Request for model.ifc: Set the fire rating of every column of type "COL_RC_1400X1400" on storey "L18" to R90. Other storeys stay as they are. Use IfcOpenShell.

First a look at what the model holds.

```python
import ifcopenshell
import ifcopenshell.util.element

model = ifcopenshell.open("model.ifc")
print(model.schema)
storey = next(s for s in model.by_type("IfcBuildingStorey") if s.Name == "L18")
columns = [e for e in ifcopenshell.util.element.get_decomposition(storey) if e.is_a("IfcColumn")]
seen = {}
for e in columns:
    element_type = ifcopenshell.util.element.get_type(e)
    key = (element_type.Name if element_type != e and element_type else None, ifcopenshell.util.element.get_pset(e, "Pset_ColumnCommon", "FireRating"))
    seen[key] = seen.get(key, 0) + 1
for (name, value), count in sorted(seen.items(), key=str):
    print(count, "x", name, "|", value)
```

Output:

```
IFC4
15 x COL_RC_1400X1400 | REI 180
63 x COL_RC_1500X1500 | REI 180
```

```python
import ifcopenshell
import ifcopenshell.api.pset
import ifcopenshell.util.element

model = ifcopenshell.open("model.ifc")

storey = next(s for s in model.by_type("IfcBuildingStorey") if s.Name == "L18")
columns = [e for e in ifcopenshell.util.element.get_decomposition(storey) if e.is_a("IfcColumn")]

count = 0
for e in columns:
    element_type = ifcopenshell.util.element.get_type(e)
    if element_type in (None, e) or element_type.Name != "COL_RC_1400X1400":
        continue
    found = ifcopenshell.util.element.get_pset(e, "Pset_ColumnCommon", should_inherit=False)
    if found:
        pset = model.by_id(found["id"])
        if len(ifcopenshell.util.element.get_elements_by_pset(pset)) > 1:
            pset = ifcopenshell.api.pset.unshare_pset(model, products=[e], pset=pset)[0]
    else:
        pset = ifcopenshell.api.pset.add_pset(model, product=e, name="Pset_ColumnCommon")
    ifcopenshell.api.pset.edit_pset(model, pset=pset, properties={"FireRating": "R90"})
    count += 1

print(count, "columns updated")

model.write("model-out.ifc")
```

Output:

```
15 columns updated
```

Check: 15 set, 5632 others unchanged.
